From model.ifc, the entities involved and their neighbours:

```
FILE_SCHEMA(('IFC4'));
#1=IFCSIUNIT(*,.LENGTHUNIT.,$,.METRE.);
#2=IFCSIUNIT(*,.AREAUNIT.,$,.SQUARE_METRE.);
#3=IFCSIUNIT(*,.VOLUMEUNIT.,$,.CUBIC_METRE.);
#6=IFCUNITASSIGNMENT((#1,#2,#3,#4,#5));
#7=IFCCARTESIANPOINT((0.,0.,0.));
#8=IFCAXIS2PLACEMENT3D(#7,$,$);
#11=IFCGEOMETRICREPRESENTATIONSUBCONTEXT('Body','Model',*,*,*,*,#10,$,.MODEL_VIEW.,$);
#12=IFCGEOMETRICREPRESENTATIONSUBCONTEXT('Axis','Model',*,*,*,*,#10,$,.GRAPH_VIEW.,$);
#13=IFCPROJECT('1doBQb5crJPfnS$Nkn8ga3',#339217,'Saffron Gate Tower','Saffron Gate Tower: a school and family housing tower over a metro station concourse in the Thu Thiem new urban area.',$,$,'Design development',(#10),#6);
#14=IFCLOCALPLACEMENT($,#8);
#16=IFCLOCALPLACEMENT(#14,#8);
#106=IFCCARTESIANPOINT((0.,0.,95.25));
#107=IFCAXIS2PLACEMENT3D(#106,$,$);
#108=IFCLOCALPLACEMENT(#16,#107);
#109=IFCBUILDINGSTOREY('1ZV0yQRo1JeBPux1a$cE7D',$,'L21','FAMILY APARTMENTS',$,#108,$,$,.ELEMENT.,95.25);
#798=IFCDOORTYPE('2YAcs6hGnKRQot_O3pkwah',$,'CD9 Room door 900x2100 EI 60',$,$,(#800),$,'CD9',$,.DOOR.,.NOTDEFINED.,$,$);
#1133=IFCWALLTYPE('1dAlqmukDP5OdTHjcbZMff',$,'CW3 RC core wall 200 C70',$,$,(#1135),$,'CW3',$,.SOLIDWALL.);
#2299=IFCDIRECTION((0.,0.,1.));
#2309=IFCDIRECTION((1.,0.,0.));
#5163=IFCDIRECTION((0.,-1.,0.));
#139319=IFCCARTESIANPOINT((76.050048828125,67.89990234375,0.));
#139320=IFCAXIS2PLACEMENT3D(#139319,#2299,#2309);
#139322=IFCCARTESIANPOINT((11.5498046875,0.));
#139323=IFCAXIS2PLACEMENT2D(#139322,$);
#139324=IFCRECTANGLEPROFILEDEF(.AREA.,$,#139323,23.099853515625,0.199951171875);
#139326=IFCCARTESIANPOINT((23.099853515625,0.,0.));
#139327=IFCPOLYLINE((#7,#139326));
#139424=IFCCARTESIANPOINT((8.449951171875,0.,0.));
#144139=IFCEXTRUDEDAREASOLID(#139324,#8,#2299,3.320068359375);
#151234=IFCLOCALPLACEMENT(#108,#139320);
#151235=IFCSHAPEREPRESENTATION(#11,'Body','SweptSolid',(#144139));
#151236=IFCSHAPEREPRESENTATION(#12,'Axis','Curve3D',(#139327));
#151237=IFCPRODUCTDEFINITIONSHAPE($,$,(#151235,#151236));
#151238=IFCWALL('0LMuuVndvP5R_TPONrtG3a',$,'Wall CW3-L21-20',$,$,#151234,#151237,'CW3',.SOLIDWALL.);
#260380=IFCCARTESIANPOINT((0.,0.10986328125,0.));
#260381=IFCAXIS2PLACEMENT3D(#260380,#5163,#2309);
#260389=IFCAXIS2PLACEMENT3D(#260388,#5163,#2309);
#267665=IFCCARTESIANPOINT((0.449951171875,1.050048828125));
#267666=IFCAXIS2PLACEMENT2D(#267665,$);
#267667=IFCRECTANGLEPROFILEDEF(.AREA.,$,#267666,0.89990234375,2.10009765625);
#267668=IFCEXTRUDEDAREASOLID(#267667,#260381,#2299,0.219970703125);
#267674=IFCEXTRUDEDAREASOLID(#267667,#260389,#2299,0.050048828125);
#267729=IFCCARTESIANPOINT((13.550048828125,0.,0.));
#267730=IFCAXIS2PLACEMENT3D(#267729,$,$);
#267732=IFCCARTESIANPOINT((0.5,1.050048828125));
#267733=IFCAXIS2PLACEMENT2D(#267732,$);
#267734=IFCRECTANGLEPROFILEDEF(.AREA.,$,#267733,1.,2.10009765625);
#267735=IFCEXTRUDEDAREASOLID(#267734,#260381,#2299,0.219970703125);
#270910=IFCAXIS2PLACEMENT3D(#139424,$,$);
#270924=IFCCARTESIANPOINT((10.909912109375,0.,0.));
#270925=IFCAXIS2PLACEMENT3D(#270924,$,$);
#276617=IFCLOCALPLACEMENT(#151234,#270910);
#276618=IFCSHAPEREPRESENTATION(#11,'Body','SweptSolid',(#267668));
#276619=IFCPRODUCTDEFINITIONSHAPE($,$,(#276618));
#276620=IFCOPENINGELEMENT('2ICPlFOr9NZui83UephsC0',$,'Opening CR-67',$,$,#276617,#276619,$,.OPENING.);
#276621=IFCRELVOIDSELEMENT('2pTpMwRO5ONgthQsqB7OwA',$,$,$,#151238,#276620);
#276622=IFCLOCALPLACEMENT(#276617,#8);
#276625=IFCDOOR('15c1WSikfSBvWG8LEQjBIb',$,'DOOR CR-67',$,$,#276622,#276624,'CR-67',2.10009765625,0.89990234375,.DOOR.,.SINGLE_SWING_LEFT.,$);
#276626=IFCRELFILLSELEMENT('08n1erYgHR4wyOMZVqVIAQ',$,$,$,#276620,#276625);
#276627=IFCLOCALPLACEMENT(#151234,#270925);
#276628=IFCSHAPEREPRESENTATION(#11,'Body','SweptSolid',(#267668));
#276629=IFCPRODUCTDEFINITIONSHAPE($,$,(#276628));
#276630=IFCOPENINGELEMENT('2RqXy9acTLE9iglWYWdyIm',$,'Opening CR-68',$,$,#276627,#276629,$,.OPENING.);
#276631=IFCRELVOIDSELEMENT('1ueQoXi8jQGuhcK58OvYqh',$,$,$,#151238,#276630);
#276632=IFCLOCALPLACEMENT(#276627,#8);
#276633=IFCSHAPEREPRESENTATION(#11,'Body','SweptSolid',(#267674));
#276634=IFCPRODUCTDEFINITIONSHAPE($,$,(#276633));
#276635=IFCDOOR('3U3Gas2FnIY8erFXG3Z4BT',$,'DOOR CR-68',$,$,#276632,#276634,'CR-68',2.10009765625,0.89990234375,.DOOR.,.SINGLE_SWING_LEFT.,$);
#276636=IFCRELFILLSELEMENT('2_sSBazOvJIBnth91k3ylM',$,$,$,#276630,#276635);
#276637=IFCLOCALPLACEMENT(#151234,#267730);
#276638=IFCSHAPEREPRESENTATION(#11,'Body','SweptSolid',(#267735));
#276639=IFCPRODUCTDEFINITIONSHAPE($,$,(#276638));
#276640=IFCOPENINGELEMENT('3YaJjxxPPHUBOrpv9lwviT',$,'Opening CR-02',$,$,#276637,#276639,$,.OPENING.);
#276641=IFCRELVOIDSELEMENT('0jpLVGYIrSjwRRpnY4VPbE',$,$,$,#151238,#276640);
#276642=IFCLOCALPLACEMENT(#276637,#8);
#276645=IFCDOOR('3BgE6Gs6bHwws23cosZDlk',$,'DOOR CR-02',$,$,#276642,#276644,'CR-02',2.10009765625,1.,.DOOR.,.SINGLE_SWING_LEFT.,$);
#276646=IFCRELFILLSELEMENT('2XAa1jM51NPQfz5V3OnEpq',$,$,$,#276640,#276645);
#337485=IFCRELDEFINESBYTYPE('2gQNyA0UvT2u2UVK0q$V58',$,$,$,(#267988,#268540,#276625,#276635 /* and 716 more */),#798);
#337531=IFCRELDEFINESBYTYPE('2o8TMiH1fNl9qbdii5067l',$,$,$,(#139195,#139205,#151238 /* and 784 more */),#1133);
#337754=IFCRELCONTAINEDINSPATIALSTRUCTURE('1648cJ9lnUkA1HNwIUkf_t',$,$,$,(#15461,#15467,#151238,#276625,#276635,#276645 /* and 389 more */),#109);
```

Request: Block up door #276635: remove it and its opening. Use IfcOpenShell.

```python
import ifcopenshell
import ifcopenshell.api.feature
import ifcopenshell.api.root
import ifcopenshell.geom
import ifcopenshell.util.shape

model = ifcopenshell.open("model.ifc")
settings = ifcopenshell.geom.settings()


def volume(element):
    """Net volume in cubic metres, openings subtracted."""
    shape = ifcopenshell.geom.create_shape(settings, element)
    return ifcopenshell.util.shape.get_volume(shape.geometry)


door = model.by_id(276635)
opening = door.FillsVoids[0].RelatingOpeningElement
wall = opening.VoidsElements[0].RelatingBuildingElement
before = volume(wall)

ifcopenshell.api.root.remove_product(model, product=door)
ifcopenshell.api.feature.remove_feature(model, feature=opening)

after = volume(wall)

print(f"wall volume {before:.3f} -> {after:.3f} m3")

model.write("model_v2.ifc")
```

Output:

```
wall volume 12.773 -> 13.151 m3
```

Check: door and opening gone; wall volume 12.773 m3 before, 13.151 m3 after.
